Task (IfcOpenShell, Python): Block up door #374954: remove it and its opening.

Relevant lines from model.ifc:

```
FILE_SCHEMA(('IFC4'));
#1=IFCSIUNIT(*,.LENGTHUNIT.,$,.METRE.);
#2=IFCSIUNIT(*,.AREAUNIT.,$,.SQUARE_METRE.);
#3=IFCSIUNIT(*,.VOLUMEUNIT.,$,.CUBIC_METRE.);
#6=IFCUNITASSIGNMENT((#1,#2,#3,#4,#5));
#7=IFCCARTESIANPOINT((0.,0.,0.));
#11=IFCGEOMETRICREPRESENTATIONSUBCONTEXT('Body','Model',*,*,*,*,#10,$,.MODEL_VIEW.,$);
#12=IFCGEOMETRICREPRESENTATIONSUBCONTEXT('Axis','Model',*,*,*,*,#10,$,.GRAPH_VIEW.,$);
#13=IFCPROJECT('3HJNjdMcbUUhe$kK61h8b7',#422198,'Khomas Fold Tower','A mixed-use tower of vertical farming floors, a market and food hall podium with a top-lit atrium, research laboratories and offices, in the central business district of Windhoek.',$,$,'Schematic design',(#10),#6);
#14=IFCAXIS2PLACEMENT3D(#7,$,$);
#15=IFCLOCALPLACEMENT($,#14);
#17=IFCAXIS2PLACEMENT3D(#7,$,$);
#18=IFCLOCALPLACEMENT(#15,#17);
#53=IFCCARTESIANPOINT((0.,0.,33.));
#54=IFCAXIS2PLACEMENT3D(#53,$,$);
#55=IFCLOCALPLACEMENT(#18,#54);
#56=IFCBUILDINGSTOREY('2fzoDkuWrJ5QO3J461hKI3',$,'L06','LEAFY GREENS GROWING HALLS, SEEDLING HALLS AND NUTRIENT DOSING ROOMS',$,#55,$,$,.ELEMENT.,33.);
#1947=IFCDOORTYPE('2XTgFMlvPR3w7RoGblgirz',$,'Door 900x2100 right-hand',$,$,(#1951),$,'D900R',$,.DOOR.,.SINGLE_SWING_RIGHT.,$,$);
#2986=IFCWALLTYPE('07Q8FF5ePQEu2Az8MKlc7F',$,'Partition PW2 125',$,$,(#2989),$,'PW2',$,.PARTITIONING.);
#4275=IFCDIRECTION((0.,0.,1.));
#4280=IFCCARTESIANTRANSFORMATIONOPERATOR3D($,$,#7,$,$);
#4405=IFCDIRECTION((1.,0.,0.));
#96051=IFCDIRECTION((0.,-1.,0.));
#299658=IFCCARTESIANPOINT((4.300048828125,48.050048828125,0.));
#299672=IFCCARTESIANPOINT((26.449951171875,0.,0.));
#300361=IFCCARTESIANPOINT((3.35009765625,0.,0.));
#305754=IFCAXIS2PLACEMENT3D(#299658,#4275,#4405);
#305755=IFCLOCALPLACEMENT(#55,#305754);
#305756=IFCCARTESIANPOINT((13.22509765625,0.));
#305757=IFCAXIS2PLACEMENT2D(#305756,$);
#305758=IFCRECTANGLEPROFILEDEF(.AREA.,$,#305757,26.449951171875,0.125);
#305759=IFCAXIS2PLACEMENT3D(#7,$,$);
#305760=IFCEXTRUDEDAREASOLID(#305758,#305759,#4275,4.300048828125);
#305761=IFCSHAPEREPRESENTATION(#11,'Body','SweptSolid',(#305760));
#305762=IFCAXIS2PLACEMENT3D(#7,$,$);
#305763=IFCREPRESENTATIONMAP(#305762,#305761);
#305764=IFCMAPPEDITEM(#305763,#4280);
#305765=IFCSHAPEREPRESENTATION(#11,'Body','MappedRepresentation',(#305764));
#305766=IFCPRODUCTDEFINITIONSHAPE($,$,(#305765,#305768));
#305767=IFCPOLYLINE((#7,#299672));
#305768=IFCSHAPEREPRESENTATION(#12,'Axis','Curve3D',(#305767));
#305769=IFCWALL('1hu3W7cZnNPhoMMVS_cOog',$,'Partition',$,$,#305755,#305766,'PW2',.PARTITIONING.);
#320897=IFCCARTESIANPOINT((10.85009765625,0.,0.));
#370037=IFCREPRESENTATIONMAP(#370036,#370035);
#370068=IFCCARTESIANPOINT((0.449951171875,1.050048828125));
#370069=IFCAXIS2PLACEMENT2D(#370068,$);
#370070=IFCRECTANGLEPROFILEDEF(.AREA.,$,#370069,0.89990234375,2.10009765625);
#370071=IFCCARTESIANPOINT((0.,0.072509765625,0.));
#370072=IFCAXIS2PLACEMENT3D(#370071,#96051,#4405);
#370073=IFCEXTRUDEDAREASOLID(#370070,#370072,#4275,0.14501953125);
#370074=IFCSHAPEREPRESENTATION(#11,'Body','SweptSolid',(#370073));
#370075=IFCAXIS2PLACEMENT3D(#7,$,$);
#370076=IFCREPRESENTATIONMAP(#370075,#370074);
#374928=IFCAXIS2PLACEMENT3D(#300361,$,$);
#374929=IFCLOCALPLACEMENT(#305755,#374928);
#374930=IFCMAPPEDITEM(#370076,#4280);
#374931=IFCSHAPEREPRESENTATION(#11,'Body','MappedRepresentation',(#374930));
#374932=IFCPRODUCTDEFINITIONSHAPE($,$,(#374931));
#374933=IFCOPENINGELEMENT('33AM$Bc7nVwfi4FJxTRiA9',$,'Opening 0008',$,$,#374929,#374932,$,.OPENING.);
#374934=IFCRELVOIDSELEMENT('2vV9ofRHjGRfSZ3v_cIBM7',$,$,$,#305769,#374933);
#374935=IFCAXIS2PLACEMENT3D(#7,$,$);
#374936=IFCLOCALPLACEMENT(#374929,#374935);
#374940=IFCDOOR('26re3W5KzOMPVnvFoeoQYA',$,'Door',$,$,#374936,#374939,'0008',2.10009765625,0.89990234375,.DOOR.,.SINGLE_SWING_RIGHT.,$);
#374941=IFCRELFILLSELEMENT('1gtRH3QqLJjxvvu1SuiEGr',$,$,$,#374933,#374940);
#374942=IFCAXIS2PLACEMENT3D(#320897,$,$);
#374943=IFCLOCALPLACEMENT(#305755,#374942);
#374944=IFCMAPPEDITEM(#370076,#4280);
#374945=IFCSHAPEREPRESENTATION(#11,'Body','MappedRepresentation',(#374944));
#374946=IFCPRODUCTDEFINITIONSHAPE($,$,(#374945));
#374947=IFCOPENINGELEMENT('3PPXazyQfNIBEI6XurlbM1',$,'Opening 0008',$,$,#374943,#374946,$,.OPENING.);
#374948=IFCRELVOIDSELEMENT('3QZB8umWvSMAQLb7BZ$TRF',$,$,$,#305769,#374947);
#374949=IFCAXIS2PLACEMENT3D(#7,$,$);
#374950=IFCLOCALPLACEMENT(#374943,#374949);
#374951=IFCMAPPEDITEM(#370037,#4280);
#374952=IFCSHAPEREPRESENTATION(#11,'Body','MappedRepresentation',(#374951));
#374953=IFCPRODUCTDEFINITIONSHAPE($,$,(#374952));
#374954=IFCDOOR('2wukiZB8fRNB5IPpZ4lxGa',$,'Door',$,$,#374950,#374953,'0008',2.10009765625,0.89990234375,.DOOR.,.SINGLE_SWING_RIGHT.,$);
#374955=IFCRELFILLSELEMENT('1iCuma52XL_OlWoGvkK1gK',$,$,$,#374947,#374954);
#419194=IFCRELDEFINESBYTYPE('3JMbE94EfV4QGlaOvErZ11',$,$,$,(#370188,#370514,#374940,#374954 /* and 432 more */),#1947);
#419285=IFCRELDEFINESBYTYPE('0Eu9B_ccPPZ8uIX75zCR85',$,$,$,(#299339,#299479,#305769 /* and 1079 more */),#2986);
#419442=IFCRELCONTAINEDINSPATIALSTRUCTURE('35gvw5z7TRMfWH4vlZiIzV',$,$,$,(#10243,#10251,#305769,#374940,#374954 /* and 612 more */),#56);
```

```python
import ifcopenshell
import ifcopenshell.api.feature
import ifcopenshell.api.root
import ifcopenshell.geom
import ifcopenshell.util.shape

model = ifcopenshell.open("model.ifc")
settings = ifcopenshell.geom.settings()


def volume(element):
    """Net volume in cubic metres, openings subtracted."""
    shape = ifcopenshell.geom.create_shape(settings, element)
    return ifcopenshell.util.shape.get_volume(shape.geometry)


door = model.by_guid("2wukiZB8fRNB5IPpZ4lxGa")
opening = door.FillsVoids[0].RelatingOpeningElement
wall = opening.VoidsElements[0].RelatingBuildingElement
before = volume(wall)

ifcopenshell.api.root.remove_product(model, product=door)
ifcopenshell.api.feature.remove_feature(model, feature=opening)

after = volume(wall)

print(f"wall volume {before:.3f} -> {after:.3f} m3")

model.write("model_rev.ifc")
```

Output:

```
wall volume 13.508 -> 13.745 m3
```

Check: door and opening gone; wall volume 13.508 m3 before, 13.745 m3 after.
